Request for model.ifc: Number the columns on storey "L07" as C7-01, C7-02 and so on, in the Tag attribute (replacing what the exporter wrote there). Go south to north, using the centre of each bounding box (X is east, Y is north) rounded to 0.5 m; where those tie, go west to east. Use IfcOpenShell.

First a look at what the model holds.

```python
import ifcopenshell
import ifcopenshell.util.element
import ifcopenshell.util.placement

model = ifcopenshell.open("model.ifc")
print(model.schema)
storey = next(s for s in model.by_type("IfcBuildingStorey") if s.Name == "L07")
columns = [e for e in ifcopenshell.util.element.get_decomposition(storey) if e.is_a("IfcColumn")]
for e in sorted(columns, key=lambda e: e.id()):
    origin = ifcopenshell.util.placement.get_local_placement(e.ObjectPlacement)[:3, 3]
    print(e.id(), e.Tag, e.Name, origin.round(2) + 0.0, sep=" | ")
```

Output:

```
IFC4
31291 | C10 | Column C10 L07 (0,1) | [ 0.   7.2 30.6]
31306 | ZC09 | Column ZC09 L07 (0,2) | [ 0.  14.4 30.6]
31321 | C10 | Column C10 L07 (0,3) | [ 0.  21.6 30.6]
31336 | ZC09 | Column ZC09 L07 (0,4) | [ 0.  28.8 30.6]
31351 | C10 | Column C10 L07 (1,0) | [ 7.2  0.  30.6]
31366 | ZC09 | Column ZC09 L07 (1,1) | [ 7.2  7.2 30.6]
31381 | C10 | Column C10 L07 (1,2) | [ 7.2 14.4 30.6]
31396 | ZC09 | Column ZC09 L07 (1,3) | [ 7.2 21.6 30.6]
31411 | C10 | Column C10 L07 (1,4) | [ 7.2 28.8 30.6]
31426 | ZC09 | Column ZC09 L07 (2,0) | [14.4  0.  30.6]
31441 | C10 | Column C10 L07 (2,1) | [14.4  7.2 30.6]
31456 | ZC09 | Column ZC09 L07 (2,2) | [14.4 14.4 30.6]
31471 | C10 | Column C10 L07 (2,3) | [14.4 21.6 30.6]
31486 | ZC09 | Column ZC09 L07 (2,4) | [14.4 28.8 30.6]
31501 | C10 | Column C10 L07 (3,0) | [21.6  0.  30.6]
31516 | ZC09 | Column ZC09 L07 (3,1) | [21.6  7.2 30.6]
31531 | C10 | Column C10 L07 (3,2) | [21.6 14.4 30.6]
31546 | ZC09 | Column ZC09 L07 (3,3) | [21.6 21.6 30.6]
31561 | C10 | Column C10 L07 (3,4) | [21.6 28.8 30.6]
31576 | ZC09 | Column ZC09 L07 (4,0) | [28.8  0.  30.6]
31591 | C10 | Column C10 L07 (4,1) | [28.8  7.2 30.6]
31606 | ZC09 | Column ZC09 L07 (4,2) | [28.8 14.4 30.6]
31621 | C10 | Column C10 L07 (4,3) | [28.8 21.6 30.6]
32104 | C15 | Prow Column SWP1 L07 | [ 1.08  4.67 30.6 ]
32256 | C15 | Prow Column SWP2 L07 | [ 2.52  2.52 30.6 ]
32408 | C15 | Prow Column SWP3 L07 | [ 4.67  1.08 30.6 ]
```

```python
import ifcopenshell
import ifcopenshell.geom
import ifcopenshell.util.element
import ifcopenshell.util.shape

model = ifcopenshell.open("model.ifc")
settings = ifcopenshell.geom.settings()
settings.set("use-world-coords", True)


def centre(element):
    shape = ifcopenshell.geom.create_shape(settings, element)
    return ifcopenshell.util.shape.get_bbox_centroid(shape.geometry)


storey = next(s for s in model.by_type("IfcBuildingStorey") if s.Name == "L07")
columns = [e for e in ifcopenshell.util.element.get_decomposition(storey) if e.is_a("IfcColumn")]

# Insertion points can sit at a corner or the storey origin, so sort by the geometry (in metres).
centres = {e: centre(e) for e in columns}
columns.sort(key=lambda e: (round(centres[e][1] / 0.5), centres[e][0]))

for i, e in enumerate(columns, start=1):
    number = f"C7-{i:02d}"
    e.Tag = number
    print(e.id(), number)

model.write("model_v2.ifc")
```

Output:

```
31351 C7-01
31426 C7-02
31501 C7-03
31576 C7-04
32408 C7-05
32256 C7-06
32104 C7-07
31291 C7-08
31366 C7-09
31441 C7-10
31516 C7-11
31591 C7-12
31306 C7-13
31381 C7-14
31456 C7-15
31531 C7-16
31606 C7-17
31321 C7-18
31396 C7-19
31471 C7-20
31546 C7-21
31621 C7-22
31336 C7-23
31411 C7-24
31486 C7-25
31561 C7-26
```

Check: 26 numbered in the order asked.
